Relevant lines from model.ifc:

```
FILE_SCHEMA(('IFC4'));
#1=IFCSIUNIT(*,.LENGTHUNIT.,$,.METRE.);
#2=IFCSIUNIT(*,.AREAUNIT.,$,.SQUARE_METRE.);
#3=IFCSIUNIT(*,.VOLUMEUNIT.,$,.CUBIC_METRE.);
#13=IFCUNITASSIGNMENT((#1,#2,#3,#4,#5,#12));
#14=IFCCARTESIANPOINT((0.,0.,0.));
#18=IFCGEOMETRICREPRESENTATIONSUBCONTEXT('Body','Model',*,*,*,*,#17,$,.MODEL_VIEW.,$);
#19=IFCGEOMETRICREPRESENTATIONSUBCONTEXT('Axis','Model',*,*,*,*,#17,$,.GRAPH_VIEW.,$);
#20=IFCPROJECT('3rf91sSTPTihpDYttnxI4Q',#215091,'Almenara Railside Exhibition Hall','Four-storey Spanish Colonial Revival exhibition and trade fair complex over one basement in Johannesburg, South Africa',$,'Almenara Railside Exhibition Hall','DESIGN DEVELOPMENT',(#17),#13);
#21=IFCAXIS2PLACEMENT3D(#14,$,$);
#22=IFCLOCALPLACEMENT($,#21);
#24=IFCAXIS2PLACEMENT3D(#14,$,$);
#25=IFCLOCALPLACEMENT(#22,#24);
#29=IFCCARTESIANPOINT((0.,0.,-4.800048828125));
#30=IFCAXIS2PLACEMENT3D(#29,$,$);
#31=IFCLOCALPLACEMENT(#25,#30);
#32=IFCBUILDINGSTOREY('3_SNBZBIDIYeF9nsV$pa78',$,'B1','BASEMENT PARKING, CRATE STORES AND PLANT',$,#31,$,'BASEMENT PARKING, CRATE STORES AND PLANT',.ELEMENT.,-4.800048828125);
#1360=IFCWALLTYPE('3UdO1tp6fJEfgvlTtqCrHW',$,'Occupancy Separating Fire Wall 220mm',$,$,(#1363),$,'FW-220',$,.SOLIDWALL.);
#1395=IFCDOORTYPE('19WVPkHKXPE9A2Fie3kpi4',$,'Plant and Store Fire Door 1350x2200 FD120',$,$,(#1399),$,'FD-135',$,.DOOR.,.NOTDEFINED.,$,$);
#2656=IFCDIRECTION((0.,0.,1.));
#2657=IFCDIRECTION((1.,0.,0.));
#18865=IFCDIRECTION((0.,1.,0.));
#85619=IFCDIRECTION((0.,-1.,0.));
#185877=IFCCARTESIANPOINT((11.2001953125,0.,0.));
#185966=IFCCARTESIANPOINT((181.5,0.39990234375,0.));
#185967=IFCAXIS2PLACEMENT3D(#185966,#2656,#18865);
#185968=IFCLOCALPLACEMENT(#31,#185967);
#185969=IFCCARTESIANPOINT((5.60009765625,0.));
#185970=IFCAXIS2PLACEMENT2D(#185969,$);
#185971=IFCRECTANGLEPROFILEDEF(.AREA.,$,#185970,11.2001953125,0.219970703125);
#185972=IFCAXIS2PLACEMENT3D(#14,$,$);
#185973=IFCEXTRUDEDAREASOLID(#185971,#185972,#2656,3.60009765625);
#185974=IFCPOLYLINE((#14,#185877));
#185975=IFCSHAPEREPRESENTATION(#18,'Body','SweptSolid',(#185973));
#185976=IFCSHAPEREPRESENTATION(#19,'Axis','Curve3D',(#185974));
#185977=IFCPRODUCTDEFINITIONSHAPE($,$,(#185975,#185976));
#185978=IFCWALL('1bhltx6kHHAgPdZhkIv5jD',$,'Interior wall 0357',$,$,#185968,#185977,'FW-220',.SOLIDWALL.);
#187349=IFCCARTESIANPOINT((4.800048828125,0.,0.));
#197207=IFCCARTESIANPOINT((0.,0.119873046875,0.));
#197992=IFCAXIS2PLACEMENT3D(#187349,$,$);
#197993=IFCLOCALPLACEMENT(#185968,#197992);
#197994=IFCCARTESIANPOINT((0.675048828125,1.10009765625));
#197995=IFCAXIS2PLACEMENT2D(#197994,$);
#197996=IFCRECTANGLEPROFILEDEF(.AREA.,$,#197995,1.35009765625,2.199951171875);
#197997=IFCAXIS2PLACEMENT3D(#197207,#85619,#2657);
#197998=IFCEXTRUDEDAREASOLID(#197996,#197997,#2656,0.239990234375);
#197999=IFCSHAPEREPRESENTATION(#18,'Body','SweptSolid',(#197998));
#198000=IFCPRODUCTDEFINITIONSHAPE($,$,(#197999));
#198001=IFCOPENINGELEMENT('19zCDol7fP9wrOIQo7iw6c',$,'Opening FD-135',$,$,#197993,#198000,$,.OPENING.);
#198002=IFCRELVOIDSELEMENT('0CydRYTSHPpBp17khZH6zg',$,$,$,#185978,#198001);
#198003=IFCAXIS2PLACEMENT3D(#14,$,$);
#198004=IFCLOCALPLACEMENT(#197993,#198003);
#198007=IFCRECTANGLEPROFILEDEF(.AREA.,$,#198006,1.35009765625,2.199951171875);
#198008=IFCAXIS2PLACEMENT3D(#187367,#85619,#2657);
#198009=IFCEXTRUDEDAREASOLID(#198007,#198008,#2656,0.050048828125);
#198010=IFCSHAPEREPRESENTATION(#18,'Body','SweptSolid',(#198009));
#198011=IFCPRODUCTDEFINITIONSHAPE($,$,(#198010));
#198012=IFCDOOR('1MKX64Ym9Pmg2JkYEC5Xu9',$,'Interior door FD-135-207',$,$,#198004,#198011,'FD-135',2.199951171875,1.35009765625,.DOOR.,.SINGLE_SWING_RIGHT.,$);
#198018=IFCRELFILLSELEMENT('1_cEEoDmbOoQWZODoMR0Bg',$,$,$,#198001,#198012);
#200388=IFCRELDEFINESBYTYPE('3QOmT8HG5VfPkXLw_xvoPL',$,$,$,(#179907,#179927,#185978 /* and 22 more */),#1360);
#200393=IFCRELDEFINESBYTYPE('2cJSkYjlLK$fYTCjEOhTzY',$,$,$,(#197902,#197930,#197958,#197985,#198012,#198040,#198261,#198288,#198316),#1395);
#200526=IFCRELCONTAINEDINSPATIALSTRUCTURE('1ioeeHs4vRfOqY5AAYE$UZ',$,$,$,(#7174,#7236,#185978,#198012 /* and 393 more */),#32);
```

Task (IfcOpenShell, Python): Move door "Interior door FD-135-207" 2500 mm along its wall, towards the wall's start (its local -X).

```python
import ifcopenshell
import ifcopenshell.api.geometry
import ifcopenshell.util.placement
import ifcopenshell.util.unit

model = ifcopenshell.open("model.ifc")
unit_scale = ifcopenshell.util.unit.calculate_unit_scale(model)

door = model.by_guid("1MKX64Ym9Pmg2JkYEC5Xu9")
opening = door.FillsVoids[0].RelatingOpeningElement
wall = opening.VoidsElements[0].RelatingBuildingElement

wall_matrix = ifcopenshell.util.placement.get_local_placement(wall.ObjectPlacement)
shift = wall_matrix[:3, 0] * -2.5 / unit_scale
before = ifcopenshell.util.placement.get_local_placement(door.ObjectPlacement)[:3, 3].copy()

# The door is placed relative to its opening, so it follows when the opening moves.
matrix = ifcopenshell.util.placement.get_local_placement(opening.ObjectPlacement)
matrix[:3, 3] += shift
ifcopenshell.api.geometry.edit_object_placement(
    model, product=opening, matrix=matrix, is_si=False, should_transform_children=True
)

after = ifcopenshell.util.placement.get_local_placement(door.ObjectPlacement)[:3, 3]
print("door moved by", (after - before).round(3) + 0.0)

model.write("model_edited.ifc")
```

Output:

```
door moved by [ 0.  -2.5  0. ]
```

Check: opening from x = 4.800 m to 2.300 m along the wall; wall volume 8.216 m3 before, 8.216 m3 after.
